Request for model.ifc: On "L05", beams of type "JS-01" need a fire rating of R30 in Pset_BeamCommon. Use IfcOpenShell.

First a look at what the model holds.

```python
import ifcopenshell
import ifcopenshell.util.element

model = ifcopenshell.open("model.ifc")
print(model.schema)
storey = next(s for s in model.by_type("IfcBuildingStorey") if s.Name == "L05")
beams = [e for e in ifcopenshell.util.element.get_decomposition(storey) if e.is_a("IfcBeam")]
seen = {}
for e in beams:
    element_type = ifcopenshell.util.element.get_type(e)
    key = (element_type.Name if element_type != e and element_type else None, ifcopenshell.util.element.get_pset(e, "Pset_BeamCommon", "FireRating"))
    seen[key] = seen.get(key, 0) + 1
for (name, value), count in sorted(seen.items(), key=str):
    print(count, "x", name, "|", value)
```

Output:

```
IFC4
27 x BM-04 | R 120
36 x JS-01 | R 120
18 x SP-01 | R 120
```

```python
import ifcopenshell
import ifcopenshell.api.pset
import ifcopenshell.util.element

model = ifcopenshell.open("model.ifc")

storey = next(s for s in model.by_type("IfcBuildingStorey") if s.Name == "L05")
beams = [e for e in ifcopenshell.util.element.get_decomposition(storey) if e.is_a("IfcBeam")]

count = 0
for e in beams:
    element_type = ifcopenshell.util.element.get_type(e)
    if element_type in (None, e) or element_type.Name != "JS-01":
        continue
    # add_pset returns the element's existing set when there is one.
    pset = ifcopenshell.api.pset.add_pset(model, product=e, name="Pset_BeamCommon")
    ifcopenshell.api.pset.edit_pset(model, pset=pset, properties={"FireRating": "R30"})
    count += 1

print(count, "beams updated")

model.write("model_edited.ifc")
```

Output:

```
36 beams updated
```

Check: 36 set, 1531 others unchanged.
